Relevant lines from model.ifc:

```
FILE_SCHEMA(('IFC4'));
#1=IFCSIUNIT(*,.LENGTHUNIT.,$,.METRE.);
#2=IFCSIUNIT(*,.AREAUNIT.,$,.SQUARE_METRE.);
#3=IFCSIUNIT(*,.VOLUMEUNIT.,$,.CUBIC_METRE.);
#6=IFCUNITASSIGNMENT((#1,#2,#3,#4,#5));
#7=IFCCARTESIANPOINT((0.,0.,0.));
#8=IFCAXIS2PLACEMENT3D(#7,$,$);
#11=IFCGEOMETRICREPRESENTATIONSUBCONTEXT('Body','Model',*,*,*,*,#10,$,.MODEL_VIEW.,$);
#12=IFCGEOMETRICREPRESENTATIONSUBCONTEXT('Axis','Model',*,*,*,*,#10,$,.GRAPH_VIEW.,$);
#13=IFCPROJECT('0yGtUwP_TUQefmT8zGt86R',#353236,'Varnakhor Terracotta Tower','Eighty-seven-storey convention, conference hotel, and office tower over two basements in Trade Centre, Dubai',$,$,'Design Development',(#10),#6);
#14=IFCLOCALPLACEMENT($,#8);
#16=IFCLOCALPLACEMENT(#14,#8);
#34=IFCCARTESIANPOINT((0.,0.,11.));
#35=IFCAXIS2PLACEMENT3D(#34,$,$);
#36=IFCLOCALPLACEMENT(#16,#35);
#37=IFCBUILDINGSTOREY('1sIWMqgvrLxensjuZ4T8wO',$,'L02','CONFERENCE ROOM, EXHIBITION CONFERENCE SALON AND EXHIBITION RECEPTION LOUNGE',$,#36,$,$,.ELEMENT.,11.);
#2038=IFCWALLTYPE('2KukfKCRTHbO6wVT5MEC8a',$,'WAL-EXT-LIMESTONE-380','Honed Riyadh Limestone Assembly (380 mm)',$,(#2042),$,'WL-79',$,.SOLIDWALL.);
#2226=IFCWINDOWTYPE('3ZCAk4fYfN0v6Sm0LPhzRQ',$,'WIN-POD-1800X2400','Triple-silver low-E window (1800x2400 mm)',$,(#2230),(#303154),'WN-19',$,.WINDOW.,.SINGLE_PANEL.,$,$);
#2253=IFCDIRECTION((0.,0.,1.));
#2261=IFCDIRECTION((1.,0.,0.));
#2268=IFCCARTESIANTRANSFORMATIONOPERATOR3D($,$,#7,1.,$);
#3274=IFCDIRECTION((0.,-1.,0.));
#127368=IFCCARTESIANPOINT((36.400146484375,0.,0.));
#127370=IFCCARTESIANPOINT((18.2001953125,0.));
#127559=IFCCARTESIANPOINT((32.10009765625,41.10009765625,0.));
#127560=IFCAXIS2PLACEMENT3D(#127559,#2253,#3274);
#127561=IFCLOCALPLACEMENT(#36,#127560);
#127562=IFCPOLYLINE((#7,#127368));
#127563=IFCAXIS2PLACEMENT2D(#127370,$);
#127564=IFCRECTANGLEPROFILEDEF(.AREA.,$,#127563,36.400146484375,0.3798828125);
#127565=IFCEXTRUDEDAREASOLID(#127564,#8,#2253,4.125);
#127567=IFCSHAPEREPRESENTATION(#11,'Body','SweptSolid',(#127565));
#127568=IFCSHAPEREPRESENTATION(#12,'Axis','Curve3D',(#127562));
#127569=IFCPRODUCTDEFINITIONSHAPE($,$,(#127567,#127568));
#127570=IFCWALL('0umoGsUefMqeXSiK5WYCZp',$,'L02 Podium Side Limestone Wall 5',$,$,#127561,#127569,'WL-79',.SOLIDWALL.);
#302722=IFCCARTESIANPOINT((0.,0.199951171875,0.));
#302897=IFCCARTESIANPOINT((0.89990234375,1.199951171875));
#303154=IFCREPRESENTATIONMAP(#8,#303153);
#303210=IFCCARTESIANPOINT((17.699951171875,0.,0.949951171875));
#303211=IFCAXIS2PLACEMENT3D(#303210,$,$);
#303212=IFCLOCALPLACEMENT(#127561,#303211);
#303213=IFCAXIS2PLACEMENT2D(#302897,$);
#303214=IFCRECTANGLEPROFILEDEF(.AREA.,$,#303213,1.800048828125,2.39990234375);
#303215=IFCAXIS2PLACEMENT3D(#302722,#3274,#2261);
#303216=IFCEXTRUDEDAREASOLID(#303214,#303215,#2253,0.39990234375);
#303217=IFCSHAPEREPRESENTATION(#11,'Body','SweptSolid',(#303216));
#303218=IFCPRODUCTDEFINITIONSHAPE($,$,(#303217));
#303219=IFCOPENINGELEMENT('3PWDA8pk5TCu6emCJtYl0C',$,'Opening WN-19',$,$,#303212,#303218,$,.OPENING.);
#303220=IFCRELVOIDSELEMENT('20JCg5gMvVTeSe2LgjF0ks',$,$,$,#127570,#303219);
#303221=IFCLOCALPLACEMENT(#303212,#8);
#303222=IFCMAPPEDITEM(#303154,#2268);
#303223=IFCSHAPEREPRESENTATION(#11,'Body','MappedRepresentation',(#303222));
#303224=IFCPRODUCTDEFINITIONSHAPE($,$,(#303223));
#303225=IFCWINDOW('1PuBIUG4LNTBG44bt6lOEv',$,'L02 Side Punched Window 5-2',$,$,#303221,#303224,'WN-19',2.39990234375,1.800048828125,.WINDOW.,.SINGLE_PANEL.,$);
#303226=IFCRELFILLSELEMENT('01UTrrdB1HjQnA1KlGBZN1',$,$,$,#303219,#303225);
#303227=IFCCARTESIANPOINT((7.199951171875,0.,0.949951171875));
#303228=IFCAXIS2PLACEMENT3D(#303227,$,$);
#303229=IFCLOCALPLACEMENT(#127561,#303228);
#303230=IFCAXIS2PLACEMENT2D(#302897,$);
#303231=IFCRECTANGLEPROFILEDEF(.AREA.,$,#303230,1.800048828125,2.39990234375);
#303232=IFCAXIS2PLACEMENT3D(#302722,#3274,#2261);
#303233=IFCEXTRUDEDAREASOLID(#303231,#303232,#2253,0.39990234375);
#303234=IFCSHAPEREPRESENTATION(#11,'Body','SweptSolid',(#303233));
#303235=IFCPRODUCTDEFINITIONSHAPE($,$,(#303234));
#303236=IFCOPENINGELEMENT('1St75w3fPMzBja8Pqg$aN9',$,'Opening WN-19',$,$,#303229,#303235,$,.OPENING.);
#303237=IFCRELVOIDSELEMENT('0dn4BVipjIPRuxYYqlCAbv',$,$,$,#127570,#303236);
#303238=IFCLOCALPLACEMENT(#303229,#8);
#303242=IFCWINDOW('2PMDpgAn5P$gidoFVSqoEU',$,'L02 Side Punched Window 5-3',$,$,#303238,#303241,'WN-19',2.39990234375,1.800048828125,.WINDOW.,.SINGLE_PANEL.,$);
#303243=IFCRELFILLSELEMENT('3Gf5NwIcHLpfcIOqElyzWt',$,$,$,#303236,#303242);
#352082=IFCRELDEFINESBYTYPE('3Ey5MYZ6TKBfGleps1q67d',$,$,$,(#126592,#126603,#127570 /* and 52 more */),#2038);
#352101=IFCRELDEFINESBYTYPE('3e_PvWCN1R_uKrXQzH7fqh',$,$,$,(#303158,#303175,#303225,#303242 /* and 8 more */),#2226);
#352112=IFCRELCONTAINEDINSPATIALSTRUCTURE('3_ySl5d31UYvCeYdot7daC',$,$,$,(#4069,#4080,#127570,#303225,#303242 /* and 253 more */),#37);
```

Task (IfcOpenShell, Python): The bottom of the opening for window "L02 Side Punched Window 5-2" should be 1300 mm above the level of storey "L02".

```python
import numpy as np
import ifcopenshell
import ifcopenshell.api.geometry
import ifcopenshell.geom
import ifcopenshell.util.element
import ifcopenshell.util.placement
import ifcopenshell.util.shape
import ifcopenshell.util.unit

model = ifcopenshell.open("model.ifc")
unit_scale = ifcopenshell.util.unit.calculate_unit_scale(model)

window = model.by_guid("1PuBIUG4LNTBG44bt6lOEv")
opening = window.FillsVoids[0].RelatingOpeningElement
storey = ifcopenshell.util.element.get_container(window, ifc_class="IfcBuildingStorey")
level = ifcopenshell.util.placement.get_local_placement(storey.ObjectPlacement)[2, 3]

# The opening's origin need not be at the sill, so measure its lowest point.
shape = ifcopenshell.geom.create_shape(ifcopenshell.geom.settings(), opening)
bottom = ifcopenshell.util.shape.get_shape_bottom_elevation(shape, shape.geometry) / unit_scale
dz = level + 1.3 / unit_scale - bottom

shift = np.array([0.0, 0.0, dz])
# The window is placed relative to its opening, so it follows when the opening moves.
matrix = ifcopenshell.util.placement.get_local_placement(opening.ObjectPlacement)
matrix[:3, 3] += shift
ifcopenshell.api.geometry.edit_object_placement(
    model, product=opening, matrix=matrix, is_si=False, should_transform_children=True
)

print(f"moved by {dz * unit_scale:+.3f} m")

model.write("model-out.ifc")
```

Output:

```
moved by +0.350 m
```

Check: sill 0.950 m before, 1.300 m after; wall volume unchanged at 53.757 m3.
